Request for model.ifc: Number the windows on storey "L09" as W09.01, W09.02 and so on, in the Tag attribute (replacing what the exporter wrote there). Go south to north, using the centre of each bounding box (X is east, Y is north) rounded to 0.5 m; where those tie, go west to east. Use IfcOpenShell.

First a look at what the model holds.

```python
import ifcopenshell
import ifcopenshell.util.element
import ifcopenshell.util.placement

model = ifcopenshell.open("model.ifc")
print(model.schema)
storey = next(s for s in model.by_type("IfcBuildingStorey") if s.Name == "L09")
windows = [e for e in ifcopenshell.util.element.get_decomposition(storey) if e.is_a("IfcWindow")]
for e in sorted(windows, key=lambda e: e.id()):
    origin = ifcopenshell.util.placement.get_local_placement(e.ObjectPlacement)[:3, 3]
    print(e.id(), e.Tag, e.Name, origin.round(2) + 0.0, sep=" | ")
```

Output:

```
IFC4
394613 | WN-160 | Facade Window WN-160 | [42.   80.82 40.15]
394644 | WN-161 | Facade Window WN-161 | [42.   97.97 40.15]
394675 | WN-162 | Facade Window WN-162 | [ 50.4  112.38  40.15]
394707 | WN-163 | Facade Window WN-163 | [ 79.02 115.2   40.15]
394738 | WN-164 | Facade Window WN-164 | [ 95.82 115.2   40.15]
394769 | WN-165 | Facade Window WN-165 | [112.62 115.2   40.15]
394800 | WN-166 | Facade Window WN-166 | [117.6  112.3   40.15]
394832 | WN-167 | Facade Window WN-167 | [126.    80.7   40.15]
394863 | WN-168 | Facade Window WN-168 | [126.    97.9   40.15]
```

```python
import ifcopenshell
import ifcopenshell.geom
import ifcopenshell.util.element
import ifcopenshell.util.shape

model = ifcopenshell.open("model.ifc")
settings = ifcopenshell.geom.settings()
settings.set("use-world-coords", True)


def centre(element):
    shape = ifcopenshell.geom.create_shape(settings, element)
    return ifcopenshell.util.shape.get_bbox_centroid(shape.geometry)


storey = next(s for s in model.by_type("IfcBuildingStorey") if s.Name == "L09")
windows = [e for e in ifcopenshell.util.element.get_decomposition(storey) if e.is_a("IfcWindow")]

# Insertion points can sit at a corner or the storey origin, so sort by the geometry (in metres).
centres = {e: centre(e) for e in windows}
windows.sort(key=lambda e: (round(centres[e][1] / 0.5), centres[e][0]))

for i, e in enumerate(windows, start=1):
    number = f"W09.{i:02d}"
    e.Tag = number
    print(e.id(), number)

model.write("model_updated.ifc")
```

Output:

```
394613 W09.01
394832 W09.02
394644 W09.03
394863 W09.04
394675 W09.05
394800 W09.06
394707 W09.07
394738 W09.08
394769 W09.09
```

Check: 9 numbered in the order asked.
